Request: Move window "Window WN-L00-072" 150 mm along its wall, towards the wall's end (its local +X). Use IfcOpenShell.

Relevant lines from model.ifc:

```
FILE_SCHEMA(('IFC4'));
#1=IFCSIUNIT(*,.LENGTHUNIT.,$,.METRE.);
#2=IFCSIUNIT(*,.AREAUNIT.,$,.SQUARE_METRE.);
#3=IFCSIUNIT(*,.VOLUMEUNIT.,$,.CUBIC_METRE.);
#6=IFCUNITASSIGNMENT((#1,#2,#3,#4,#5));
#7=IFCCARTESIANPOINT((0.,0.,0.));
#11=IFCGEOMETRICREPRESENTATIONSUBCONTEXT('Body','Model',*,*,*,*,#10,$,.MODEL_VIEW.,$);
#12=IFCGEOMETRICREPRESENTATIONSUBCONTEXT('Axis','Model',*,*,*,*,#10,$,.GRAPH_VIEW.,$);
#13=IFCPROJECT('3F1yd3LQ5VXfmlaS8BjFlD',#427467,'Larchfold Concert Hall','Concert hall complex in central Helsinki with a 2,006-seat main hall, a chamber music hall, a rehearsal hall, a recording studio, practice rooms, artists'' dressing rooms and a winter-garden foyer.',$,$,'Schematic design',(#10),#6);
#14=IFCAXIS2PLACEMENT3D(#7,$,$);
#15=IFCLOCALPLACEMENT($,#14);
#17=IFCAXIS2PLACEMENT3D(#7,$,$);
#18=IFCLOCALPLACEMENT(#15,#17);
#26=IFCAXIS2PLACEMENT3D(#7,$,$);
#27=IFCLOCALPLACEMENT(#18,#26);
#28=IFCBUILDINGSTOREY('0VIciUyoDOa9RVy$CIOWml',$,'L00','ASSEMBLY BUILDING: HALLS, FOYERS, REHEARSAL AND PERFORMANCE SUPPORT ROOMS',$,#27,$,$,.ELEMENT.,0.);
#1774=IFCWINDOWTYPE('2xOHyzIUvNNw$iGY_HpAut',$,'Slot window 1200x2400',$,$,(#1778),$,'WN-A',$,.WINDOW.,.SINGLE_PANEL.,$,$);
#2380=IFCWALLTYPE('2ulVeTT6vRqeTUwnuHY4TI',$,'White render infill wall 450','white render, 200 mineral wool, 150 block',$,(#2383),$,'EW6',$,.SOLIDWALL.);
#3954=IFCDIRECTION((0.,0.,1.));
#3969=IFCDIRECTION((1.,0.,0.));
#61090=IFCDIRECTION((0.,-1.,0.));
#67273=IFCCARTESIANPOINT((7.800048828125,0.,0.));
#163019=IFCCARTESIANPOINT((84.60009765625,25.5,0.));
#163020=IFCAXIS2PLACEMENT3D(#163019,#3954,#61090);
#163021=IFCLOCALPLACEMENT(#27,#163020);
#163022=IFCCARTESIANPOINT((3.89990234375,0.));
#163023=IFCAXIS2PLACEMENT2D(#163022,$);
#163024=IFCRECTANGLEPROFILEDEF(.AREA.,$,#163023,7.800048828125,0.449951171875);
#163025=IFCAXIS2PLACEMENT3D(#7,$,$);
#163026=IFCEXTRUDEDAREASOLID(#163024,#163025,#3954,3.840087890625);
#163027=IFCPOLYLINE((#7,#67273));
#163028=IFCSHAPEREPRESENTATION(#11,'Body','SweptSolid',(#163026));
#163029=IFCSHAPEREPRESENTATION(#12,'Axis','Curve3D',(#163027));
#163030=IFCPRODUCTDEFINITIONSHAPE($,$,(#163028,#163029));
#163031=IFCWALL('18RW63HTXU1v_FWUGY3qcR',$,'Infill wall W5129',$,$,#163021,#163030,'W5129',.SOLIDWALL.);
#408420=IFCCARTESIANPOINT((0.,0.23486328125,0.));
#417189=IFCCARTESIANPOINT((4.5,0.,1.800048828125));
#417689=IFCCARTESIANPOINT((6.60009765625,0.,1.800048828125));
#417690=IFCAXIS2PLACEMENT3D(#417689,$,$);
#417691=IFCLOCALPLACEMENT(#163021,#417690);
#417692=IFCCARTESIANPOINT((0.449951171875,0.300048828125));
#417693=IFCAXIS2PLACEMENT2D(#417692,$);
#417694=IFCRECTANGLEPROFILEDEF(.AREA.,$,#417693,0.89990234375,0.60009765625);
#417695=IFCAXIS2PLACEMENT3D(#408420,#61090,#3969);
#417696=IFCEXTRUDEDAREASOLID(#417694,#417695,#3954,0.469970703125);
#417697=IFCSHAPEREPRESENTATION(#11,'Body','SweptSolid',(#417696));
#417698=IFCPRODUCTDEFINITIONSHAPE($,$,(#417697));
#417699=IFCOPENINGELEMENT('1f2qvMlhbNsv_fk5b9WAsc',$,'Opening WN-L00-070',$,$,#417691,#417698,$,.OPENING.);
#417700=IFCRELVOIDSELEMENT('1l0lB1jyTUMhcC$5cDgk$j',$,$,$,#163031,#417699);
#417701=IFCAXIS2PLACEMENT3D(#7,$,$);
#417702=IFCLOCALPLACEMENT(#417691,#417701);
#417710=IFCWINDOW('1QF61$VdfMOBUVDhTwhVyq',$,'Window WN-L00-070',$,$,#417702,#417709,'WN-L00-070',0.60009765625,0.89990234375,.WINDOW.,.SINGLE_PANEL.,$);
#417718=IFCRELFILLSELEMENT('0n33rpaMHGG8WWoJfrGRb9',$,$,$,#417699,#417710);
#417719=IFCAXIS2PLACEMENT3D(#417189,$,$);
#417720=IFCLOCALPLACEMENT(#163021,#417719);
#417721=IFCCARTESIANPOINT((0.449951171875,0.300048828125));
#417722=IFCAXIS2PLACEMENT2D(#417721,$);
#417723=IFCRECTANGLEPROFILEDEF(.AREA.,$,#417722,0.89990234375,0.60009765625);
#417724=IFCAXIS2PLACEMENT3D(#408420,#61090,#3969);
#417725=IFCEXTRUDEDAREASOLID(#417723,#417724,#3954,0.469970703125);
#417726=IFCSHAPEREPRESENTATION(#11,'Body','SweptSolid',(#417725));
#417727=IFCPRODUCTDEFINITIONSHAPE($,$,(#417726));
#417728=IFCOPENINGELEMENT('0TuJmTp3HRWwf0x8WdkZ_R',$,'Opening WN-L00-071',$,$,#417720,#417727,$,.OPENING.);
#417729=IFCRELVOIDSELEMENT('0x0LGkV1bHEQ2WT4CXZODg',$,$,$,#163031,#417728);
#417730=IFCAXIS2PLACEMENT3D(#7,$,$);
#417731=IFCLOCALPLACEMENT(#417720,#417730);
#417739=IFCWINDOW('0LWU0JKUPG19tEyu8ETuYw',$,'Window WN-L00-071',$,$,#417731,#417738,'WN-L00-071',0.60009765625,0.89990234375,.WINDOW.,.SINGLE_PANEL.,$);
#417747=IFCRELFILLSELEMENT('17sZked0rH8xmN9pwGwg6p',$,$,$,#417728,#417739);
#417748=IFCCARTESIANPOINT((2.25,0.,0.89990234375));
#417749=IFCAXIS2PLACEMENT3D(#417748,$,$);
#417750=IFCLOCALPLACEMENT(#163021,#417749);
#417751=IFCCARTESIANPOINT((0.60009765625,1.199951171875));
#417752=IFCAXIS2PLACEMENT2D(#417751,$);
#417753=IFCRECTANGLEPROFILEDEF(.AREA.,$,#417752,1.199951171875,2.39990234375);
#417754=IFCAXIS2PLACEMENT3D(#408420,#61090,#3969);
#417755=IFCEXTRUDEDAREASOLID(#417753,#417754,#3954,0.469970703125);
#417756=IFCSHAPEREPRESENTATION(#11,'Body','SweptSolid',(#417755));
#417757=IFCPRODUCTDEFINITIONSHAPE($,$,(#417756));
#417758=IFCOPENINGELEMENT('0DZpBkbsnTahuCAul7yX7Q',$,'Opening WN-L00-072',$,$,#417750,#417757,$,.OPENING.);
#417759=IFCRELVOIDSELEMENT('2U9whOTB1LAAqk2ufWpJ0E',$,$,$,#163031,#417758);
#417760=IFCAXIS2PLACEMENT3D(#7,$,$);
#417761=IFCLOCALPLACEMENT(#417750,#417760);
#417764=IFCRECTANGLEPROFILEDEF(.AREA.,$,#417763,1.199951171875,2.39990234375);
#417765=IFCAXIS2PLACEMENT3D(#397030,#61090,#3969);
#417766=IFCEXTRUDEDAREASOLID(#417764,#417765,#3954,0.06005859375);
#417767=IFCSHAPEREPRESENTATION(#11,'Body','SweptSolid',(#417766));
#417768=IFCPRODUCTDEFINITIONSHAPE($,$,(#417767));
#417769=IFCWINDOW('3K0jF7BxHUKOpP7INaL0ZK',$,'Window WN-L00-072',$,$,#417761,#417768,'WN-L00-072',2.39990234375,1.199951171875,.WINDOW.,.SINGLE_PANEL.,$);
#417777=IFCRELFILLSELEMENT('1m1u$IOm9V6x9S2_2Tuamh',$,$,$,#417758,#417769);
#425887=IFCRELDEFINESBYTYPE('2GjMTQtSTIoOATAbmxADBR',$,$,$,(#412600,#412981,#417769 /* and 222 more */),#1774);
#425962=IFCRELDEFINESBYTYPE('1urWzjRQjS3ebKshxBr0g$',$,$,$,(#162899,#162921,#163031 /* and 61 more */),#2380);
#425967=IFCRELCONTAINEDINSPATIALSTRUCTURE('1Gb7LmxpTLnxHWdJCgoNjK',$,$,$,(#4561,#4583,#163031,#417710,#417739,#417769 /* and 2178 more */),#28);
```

```python
import ifcopenshell
import ifcopenshell.api.geometry
import ifcopenshell.util.placement

model = ifcopenshell.open("model.ifc")

window = model.by_id(417769)
opening = window.FillsVoids[0].RelatingOpeningElement
wall = opening.VoidsElements[0].RelatingBuildingElement

wall_matrix = ifcopenshell.util.placement.get_local_placement(wall.ObjectPlacement)
shift = wall_matrix[:3, 0] * 0.15
before = ifcopenshell.util.placement.get_local_placement(window.ObjectPlacement)[:3, 3].copy()

# The window is placed relative to its opening, so it follows when the opening moves.
matrix = ifcopenshell.util.placement.get_local_placement(opening.ObjectPlacement)
matrix[:3, 3] += shift
ifcopenshell.api.geometry.edit_object_placement(
    model, product=opening, matrix=matrix, is_si=False, should_transform_children=True
)

after = ifcopenshell.util.placement.get_local_placement(window.ObjectPlacement)[:3, 3]
print("window moved by", (after - before).round(3) + 0.0)

model.write("model_edited.ifc")
```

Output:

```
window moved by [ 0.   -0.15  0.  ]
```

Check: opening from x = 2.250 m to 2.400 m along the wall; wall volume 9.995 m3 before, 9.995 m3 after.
